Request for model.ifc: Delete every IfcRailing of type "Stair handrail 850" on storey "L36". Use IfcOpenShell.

First a look at what the model holds.

```python
import ifcopenshell
import ifcopenshell.util.element

model = ifcopenshell.open("model.ifc")
print(model.schema)
storey = next(s for s in model.by_type("IfcBuildingStorey") if s.Name == "L36")
railings = [e for e in ifcopenshell.util.element.get_decomposition(storey) if e.is_a("IfcRailing")]
seen = {}
for e in railings:
    element_type = ifcopenshell.util.element.get_type(e)
    name = element_type.Name if element_type not in (None, e) else None
    seen[name] = seen.get(name, 0) + 1
for name, count in sorted(seen.items(), key=str):
    print(count, "x", name)
```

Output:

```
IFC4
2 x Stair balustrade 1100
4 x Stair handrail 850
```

```python
import ifcopenshell
import ifcopenshell.api.root
import ifcopenshell.util.element

model = ifcopenshell.open("model.ifc")

storey = next(s for s in model.by_type("IfcBuildingStorey") if s.Name == "L36")
railings = [e for e in ifcopenshell.util.element.get_decomposition(storey) if e.is_a("IfcRailing")]
targets = [e for e in railings if (t := ifcopenshell.util.element.get_type(e)) not in (None, e) and t.Name == "Stair handrail 850"]

for e in targets:
    ifcopenshell.api.root.remove_product(model, product=e)
print(len(targets), "removed")

model.write("model_edited.ifc")
```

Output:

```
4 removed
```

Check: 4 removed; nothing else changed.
